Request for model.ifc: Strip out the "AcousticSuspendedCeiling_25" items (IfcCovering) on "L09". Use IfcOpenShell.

First a look at what the model holds.

```python
import ifcopenshell
import ifcopenshell.util.element

model = ifcopenshell.open("model.ifc")
print(model.schema)
storey = next(s for s in model.by_type("IfcBuildingStorey") if s.Name == "L09")
coverings = [e for e in ifcopenshell.util.element.get_decomposition(storey) if e.is_a("IfcCovering")]
seen = {}
for e in coverings:
    element_type = ifcopenshell.util.element.get_type(e)
    name = element_type.Name if element_type not in (None, e) else None
    seen[name] = seen.get(name, 0) + 1
for name, count in sorted(seen.items(), key=str):
    print(count, "x", name)
```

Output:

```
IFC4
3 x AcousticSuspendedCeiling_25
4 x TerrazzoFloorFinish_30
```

```python
import ifcopenshell
import ifcopenshell.api.root
import ifcopenshell.util.element

model = ifcopenshell.open("model.ifc")

storey = next(s for s in model.by_type("IfcBuildingStorey") if s.Name == "L09")
coverings = [e for e in ifcopenshell.util.element.get_decomposition(storey) if e.is_a("IfcCovering")]
targets = [e for e in coverings if (t := ifcopenshell.util.element.get_type(e)) not in (None, e) and t.Name == "AcousticSuspendedCeiling_25"]

for e in targets:
    ifcopenshell.api.root.remove_product(model, product=e)
print(len(targets), "removed")

model.write("model_rev.ifc")
```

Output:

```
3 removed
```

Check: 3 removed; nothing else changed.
